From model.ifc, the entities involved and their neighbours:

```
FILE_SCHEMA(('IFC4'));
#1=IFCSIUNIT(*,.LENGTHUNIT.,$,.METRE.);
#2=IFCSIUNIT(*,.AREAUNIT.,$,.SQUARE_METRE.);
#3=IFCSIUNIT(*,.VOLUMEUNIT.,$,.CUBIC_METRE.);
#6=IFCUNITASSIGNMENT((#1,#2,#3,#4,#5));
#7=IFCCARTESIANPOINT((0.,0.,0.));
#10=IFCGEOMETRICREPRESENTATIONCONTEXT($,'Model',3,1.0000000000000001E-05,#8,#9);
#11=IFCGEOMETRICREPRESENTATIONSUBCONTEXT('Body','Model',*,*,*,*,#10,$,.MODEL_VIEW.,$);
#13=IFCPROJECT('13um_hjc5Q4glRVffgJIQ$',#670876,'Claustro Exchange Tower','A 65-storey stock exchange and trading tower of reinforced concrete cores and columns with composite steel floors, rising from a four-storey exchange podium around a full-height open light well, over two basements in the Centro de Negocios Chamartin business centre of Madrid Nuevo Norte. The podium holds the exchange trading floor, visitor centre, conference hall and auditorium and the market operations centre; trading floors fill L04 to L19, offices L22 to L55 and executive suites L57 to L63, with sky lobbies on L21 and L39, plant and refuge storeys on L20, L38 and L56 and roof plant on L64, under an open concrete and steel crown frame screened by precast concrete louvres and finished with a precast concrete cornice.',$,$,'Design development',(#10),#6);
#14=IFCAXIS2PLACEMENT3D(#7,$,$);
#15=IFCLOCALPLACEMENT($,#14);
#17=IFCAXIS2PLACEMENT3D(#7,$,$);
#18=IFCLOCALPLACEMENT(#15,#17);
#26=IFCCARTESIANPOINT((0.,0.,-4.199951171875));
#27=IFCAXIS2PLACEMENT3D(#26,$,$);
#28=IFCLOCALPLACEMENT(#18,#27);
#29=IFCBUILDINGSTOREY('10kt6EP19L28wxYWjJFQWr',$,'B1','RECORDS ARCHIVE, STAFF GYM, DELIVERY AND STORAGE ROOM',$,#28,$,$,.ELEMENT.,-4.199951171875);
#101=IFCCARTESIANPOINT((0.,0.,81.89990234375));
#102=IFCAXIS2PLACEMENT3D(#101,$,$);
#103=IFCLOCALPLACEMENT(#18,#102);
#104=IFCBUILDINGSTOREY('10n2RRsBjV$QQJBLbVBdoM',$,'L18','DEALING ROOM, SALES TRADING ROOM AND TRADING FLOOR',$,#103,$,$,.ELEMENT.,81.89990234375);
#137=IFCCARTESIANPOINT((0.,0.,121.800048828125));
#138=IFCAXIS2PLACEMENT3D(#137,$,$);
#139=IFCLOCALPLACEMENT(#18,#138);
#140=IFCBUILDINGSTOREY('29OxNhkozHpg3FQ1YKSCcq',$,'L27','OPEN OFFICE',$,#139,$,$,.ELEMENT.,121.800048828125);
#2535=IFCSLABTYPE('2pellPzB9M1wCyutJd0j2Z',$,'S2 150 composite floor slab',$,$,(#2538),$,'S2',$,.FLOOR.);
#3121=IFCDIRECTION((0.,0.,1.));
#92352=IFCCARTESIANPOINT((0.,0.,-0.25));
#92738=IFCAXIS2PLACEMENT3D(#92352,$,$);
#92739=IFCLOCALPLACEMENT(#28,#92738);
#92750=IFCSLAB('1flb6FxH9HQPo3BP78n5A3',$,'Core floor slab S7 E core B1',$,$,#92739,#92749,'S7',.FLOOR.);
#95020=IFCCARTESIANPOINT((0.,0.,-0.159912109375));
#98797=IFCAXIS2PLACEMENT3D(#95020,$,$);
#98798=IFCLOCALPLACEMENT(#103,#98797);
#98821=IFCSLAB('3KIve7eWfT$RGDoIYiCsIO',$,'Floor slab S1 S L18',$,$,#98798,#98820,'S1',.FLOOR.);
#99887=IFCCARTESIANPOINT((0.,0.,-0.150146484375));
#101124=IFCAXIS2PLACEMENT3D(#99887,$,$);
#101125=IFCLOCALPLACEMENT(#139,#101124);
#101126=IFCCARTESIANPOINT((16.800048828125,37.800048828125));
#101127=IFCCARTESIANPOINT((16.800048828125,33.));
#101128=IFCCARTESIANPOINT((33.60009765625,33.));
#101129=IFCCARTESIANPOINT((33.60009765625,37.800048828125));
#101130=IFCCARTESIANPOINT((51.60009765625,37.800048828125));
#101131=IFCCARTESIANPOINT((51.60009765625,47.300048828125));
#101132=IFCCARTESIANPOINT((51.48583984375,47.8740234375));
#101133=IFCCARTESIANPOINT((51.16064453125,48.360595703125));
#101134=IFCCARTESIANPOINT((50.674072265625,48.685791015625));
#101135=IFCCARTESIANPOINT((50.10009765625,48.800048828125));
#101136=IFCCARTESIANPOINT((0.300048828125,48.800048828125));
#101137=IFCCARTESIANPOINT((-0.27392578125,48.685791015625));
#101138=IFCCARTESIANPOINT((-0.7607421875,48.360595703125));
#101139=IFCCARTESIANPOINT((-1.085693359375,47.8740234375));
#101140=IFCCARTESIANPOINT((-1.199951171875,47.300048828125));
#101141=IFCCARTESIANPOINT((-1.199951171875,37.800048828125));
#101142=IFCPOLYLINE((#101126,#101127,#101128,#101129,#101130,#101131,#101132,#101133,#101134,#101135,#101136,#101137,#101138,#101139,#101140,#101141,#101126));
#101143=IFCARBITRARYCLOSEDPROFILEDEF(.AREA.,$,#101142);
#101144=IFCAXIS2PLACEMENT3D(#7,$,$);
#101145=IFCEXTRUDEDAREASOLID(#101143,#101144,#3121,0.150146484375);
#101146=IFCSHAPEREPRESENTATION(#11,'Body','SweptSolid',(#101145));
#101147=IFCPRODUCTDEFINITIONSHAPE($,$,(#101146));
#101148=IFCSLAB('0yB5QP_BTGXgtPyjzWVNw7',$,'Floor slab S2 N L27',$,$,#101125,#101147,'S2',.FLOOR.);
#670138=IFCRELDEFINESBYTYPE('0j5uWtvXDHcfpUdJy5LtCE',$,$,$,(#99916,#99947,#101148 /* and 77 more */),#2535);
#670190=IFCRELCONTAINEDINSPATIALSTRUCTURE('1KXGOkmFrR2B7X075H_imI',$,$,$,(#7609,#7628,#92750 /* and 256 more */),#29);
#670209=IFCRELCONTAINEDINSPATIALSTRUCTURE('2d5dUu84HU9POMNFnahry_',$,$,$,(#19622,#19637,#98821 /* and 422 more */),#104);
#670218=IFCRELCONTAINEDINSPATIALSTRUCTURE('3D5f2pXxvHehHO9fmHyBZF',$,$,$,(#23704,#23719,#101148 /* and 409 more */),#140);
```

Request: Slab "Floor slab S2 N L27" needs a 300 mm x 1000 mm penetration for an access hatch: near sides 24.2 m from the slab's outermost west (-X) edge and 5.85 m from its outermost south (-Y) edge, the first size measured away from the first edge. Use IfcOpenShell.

```python
import numpy as np
import ifcopenshell
import ifcopenshell.api.feature
import ifcopenshell.api.geometry
import ifcopenshell.api.root
import ifcopenshell.geom
import ifcopenshell.util.placement
import ifcopenshell.util.representation
import ifcopenshell.util.shape
import ifcopenshell.util.unit

model = ifcopenshell.open("model.ifc")
unit_scale = ifcopenshell.util.unit.calculate_unit_scale(model)
settings = ifcopenshell.geom.settings()


def volume(element):
    """Net volume in cubic metres, openings subtracted."""
    shape = ifcopenshell.geom.create_shape(settings, element)
    return ifcopenshell.util.shape.get_volume(shape.geometry)


slab = model.by_id(101148)
before = volume(slab)

# Extent in the slab's own axes, in metres. The edges named are its -X and -Y sides.
slab_shape = ifcopenshell.geom.create_shape(settings, slab)
vertices = ifcopenshell.util.shape.get_vertices(slab_shape.geometry)
x_min, y_min, bottom = vertices.min(axis=0)
top = vertices[:, 2].max()

opening = ifcopenshell.api.root.create_entity(model, ifc_class="IfcOpeningElement", name="Access hatch opening", predefined_type="OPENING")
context = ifcopenshell.util.representation.get_context(model, "Model", "Body", "MODEL_VIEW")
width, depth = 0.3, 1
outline = [(0.0, 0.0), (width, 0.0), (width, depth), (0.0, depth), (0.0, 0.0)]
# Overshoot both faces by 50 mm so the cut is clean.
shape = ifcopenshell.api.geometry.add_slab_representation(
    model, context=context, depth=top - bottom + 0.1, polyline=outline
)
ifcopenshell.api.geometry.assign_representation(model, product=opening, representation=shape)

matrix = ifcopenshell.util.placement.get_local_placement(slab.ObjectPlacement)
matrix[:, 3] = matrix @ np.append(np.array([x_min + 24.2, y_min + 5.85, bottom - 0.05]) / unit_scale, 1.0)
ifcopenshell.api.geometry.edit_object_placement(model, product=opening, matrix=matrix, is_si=False)
ifcopenshell.api.feature.add_feature(model, feature=opening, element=slab)

after = volume(slab)

print(f"slab volume {before:.3f} -> {after:.3f} m3")

model.write("model_v2.ifc")
```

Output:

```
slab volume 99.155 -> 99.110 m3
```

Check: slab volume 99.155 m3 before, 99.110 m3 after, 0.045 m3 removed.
